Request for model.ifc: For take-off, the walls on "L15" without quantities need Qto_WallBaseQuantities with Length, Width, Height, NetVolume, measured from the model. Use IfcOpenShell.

First a look at what the model holds.

```python
import ifcopenshell
import ifcopenshell.util.element
import ifcopenshell.util.unit

model = ifcopenshell.open("model.ifc")
print(model.schema)
for unit_type in ("LENGTHUNIT", "AREAUNIT", "VOLUMEUNIT"):
    print(unit_type, ifcopenshell.util.unit.calculate_unit_scale(model, unit_type))
storey = next(s for s in model.by_type("IfcBuildingStorey") if s.Name == "L15")
walls = [e for e in ifcopenshell.util.element.get_decomposition(storey) if e.is_a("IfcWall")]
for e in sorted(walls, key=lambda e: e.id()):
    print(e.id(), e.is_a(), e.Name, list(ifcopenshell.util.element.get_psets(e, qtos_only=True)), sep=" | ")
```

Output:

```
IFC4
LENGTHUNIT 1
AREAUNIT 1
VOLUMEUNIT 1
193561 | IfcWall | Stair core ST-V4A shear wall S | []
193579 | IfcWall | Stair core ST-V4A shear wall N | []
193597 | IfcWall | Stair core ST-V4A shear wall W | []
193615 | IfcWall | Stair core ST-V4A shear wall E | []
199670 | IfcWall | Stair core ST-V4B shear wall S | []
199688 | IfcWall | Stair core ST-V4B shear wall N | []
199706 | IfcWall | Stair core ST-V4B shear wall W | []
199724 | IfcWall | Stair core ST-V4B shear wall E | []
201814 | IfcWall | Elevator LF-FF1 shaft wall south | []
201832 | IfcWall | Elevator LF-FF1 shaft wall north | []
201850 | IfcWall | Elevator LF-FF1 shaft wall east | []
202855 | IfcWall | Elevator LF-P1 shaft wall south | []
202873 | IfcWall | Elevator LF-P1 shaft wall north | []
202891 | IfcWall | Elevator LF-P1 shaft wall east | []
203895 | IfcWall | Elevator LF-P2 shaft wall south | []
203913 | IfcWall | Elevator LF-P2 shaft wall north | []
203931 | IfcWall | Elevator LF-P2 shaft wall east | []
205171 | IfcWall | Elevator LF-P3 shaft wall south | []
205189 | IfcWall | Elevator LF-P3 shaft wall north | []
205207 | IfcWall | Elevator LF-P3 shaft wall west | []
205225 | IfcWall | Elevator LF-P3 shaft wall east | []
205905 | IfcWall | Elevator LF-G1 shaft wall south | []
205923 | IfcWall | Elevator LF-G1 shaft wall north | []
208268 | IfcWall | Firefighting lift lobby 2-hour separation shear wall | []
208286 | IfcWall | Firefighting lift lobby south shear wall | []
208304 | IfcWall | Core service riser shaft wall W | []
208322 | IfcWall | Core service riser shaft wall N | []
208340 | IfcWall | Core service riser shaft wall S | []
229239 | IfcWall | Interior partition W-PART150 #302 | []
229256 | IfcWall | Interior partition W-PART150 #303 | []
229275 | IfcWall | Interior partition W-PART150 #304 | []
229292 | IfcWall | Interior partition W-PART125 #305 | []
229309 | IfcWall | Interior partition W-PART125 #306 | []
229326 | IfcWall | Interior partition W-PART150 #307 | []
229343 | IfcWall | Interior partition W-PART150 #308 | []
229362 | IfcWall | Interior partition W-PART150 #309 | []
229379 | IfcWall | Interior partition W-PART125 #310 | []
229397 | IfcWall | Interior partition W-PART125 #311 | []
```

```python
import ifcopenshell
import ifcopenshell.api.pset
import ifcopenshell.geom
import ifcopenshell.util.element
import ifcopenshell.util.shape
import ifcopenshell.util.unit

model = ifcopenshell.open("model.ifc")
unit_scale = ifcopenshell.util.unit.calculate_unit_scale(model)
volume_scale = ifcopenshell.util.unit.calculate_unit_scale(model, "VOLUMEUNIT")
settings = ifcopenshell.geom.settings()

storey = next(s for s in model.by_type("IfcBuildingStorey") if s.Name == "L15")
walls = [e for e in ifcopenshell.util.element.get_decomposition(storey) if e.is_a("IfcWall")]

for e in sorted(walls, key=lambda e: e.id()):
    if ifcopenshell.util.element.get_psets(e, qtos_only=True, should_inherit=False):
        continue
    # Geometry comes back in metres, in the element's own axes.
    shape = ifcopenshell.geom.create_shape(settings, e)
    values = {
        "Length": ifcopenshell.util.shape.get_x(shape.geometry) / unit_scale,
        "Width": ifcopenshell.util.shape.get_y(shape.geometry) / unit_scale,
        "Height": ifcopenshell.util.shape.get_z(shape.geometry) / unit_scale,
        "NetVolume": ifcopenshell.util.shape.get_volume(shape.geometry) / volume_scale,
    }
    qto = ifcopenshell.api.pset.add_qto(model, product=e, name="Qto_WallBaseQuantities")
    ifcopenshell.api.pset.edit_qto(model, qto=qto, properties=values)
    print(e.id(), {k: round(v, 3) for k, v in values.items()})

model.write("model_edited.ifc")
```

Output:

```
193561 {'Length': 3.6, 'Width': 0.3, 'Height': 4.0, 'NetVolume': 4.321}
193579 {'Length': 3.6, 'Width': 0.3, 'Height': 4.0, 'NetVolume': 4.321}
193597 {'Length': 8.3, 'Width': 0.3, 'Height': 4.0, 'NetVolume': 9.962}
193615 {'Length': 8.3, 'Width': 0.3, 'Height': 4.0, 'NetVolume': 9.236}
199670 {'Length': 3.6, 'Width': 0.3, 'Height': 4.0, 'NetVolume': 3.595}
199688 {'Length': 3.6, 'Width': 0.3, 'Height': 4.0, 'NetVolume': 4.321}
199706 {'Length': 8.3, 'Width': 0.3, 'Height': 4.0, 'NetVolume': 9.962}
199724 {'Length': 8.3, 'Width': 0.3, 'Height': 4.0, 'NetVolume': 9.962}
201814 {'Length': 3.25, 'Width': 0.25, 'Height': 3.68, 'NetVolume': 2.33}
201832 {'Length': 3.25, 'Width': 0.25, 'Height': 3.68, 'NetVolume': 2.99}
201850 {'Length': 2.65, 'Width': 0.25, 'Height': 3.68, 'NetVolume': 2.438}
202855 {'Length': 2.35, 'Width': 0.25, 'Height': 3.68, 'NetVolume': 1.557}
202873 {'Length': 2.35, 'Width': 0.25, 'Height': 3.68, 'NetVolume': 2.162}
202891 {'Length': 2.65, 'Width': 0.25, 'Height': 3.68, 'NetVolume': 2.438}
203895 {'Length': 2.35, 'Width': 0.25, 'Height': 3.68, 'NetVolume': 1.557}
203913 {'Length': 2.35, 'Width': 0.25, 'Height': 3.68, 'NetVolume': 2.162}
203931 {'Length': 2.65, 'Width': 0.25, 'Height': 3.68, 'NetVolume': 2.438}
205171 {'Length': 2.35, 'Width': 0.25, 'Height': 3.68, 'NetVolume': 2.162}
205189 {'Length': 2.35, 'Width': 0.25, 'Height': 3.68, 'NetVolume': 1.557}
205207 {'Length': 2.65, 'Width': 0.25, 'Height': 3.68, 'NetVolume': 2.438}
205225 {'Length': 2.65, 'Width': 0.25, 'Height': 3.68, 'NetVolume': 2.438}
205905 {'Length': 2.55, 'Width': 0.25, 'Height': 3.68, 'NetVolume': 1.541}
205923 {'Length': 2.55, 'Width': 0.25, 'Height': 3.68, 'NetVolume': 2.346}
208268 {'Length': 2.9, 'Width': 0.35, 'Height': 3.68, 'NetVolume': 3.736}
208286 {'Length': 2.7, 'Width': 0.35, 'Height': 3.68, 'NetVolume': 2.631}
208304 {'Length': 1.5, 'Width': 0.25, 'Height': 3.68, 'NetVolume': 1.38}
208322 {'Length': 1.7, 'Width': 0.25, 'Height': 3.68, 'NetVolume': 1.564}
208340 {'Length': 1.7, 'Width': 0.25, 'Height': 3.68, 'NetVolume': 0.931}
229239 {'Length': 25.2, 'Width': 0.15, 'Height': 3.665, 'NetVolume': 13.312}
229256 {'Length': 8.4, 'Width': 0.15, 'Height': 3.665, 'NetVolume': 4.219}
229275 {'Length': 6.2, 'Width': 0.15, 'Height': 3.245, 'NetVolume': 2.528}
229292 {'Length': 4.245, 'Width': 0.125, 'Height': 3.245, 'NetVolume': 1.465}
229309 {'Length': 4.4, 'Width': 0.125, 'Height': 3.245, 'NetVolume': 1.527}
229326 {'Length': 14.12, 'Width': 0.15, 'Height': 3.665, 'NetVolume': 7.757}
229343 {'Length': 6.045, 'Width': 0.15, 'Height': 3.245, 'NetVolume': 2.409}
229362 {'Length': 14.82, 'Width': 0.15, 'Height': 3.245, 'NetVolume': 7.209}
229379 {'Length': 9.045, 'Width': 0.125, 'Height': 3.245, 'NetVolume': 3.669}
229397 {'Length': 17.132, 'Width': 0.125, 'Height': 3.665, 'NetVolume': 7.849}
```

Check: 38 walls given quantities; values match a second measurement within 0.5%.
